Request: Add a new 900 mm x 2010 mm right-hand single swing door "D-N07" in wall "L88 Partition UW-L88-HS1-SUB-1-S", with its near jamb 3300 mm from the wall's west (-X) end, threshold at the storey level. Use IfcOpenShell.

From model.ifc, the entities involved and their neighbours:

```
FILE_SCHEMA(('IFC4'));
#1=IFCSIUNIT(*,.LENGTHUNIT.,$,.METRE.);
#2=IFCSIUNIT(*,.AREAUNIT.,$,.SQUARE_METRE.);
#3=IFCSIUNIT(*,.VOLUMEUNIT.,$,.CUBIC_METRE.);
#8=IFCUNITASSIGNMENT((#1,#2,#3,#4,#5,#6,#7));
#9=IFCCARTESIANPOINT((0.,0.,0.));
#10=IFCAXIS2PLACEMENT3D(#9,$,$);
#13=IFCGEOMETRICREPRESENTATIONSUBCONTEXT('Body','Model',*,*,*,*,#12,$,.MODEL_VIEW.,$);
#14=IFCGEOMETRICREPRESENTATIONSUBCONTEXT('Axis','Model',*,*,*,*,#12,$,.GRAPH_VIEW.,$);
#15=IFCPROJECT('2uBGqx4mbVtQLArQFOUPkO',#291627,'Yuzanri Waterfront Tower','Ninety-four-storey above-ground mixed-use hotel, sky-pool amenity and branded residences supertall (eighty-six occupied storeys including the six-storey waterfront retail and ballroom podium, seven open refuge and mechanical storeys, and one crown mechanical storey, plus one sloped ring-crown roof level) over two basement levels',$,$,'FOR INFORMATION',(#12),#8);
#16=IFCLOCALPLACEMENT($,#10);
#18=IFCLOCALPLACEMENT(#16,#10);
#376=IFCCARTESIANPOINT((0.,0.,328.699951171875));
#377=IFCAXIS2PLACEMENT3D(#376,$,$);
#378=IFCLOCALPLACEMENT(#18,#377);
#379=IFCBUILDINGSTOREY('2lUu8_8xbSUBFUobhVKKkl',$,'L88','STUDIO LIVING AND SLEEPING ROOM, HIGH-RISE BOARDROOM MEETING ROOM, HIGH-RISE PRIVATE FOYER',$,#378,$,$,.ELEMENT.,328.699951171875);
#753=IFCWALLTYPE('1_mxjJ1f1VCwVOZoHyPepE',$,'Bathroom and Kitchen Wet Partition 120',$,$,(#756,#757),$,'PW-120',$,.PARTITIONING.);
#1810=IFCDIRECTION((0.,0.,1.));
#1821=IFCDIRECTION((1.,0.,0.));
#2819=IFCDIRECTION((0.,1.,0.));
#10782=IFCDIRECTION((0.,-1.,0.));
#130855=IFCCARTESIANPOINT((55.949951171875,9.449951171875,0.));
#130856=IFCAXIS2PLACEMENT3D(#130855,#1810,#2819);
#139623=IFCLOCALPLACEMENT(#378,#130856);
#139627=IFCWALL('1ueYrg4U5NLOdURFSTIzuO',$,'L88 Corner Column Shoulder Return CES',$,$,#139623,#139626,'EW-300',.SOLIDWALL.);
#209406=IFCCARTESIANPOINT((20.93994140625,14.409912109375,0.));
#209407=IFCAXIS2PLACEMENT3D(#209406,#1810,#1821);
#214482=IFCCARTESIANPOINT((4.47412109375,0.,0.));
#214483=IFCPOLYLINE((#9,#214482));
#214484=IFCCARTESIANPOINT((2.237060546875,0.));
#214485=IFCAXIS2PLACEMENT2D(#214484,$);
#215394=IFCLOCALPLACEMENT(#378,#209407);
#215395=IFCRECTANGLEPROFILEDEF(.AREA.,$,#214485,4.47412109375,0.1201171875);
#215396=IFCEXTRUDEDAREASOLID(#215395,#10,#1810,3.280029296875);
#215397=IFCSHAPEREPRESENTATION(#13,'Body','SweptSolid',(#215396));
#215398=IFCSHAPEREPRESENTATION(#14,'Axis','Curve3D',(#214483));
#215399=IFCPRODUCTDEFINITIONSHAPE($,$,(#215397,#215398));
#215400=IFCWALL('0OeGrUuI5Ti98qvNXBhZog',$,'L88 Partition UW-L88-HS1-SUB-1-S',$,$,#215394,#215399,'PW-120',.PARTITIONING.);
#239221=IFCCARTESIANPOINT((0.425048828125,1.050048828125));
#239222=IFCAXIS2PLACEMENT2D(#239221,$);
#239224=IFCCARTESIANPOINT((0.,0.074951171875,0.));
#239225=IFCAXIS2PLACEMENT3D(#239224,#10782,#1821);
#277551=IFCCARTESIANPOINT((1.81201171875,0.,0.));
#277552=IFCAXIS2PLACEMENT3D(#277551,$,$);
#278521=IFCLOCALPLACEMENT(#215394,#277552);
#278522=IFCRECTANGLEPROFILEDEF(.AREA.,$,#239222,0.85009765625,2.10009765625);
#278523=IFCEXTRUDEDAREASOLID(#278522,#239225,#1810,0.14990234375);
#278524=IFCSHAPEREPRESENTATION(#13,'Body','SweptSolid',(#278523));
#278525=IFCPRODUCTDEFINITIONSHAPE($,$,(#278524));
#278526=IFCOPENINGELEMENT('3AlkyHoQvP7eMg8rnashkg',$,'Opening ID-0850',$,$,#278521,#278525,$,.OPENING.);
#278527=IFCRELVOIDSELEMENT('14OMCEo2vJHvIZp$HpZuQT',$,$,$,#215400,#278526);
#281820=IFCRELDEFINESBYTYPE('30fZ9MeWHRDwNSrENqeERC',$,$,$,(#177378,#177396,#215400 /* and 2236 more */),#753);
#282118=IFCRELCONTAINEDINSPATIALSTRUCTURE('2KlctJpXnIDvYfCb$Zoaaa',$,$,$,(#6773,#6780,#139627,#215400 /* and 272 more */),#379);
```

```python
import numpy as np
import ifcopenshell
import ifcopenshell.api.feature
import ifcopenshell.api.geometry
import ifcopenshell.api.root
import ifcopenshell.api.spatial
import ifcopenshell.geom
import ifcopenshell.util.element
import ifcopenshell.util.placement
import ifcopenshell.util.representation
import ifcopenshell.util.shape
import ifcopenshell.util.unit

model = ifcopenshell.open("model.ifc")
unit_scale = ifcopenshell.util.unit.calculate_unit_scale(model)
settings = ifcopenshell.geom.settings()


def volume(element):
    """Net volume in cubic metres, openings subtracted."""
    shape = ifcopenshell.geom.create_shape(settings, element)
    return ifcopenshell.util.shape.get_volume(shape.geometry)


wall = model.by_guid("0OeGrUuI5Ti98qvNXBhZog")
storey = ifcopenshell.util.element.get_container(wall, ifc_class="IfcBuildingStorey")
context = ifcopenshell.util.representation.get_context(model, "Model", "Body", "MODEL_VIEW")
before = volume(wall)

width, height, from_end, sill = 0.9, 2.01, 3.3, 0.0  # metres

# The wall runs along its own X axis, and the end named is its -X end.
wall_shape = ifcopenshell.geom.create_shape(settings, wall)
x, y, z = ifcopenshell.util.shape.get_vertices(wall_shape.geometry).T
start = x.min() + from_end
face, thickness = float(y.min()), float(y.max() - y.min())
wall_matrix = ifcopenshell.util.placement.get_local_placement(wall.ObjectPlacement)
level = ifcopenshell.util.placement.get_local_placement(storey.ObjectPlacement)[2, 3]


def in_wall(x, y):
    """Placement at x, y metres in the wall's axes, at sill height."""
    matrix = wall_matrix.copy()
    matrix[:, 3] = wall_matrix @ np.array([x / unit_scale, y / unit_scale, 0.0, 1.0])
    matrix[2, 3] = level + sill / unit_scale
    return matrix


# Opening: a box that overshoots both wall faces by 50 mm.
opening = ifcopenshell.api.root.create_entity(model, ifc_class="IfcOpeningElement", predefined_type="OPENING")
box = ifcopenshell.api.geometry.add_wall_representation(
    model, context=context, length=width, height=height, thickness=thickness + 0.1
)
ifcopenshell.api.geometry.assign_representation(model, product=opening, representation=box)
ifcopenshell.api.geometry.edit_object_placement(model, product=opening, matrix=in_wall(start, face - 0.05), is_si=False)
ifcopenshell.api.feature.add_feature(model, feature=opening, element=wall)

door = ifcopenshell.api.root.create_entity(model, ifc_class="IfcDoor", name="D-N07", predefined_type="DOOR")
door.OverallWidth, door.OverallHeight = width / unit_scale, height / unit_scale
door.OperationType = "SINGLE_SWING_RIGHT"
body = ifcopenshell.api.geometry.add_door_representation(
    model,
    context=context,
    overall_width=door.OverallWidth,
    overall_height=door.OverallHeight,
    operation_type="SINGLE_SWING_RIGHT",
    lining_properties={"LiningDepth": thickness / unit_scale, "ThresholdDepth": thickness / unit_scale},
)
ifcopenshell.api.geometry.assign_representation(model, product=door, representation=body)
ifcopenshell.api.spatial.assign_container(model, products=[door], relating_structure=storey)
ifcopenshell.api.feature.add_filling(model, opening=opening, element=door)

# The lining spans the wall, so the door starts at the wall face.
ifcopenshell.api.geometry.edit_object_placement(model, product=door, matrix=in_wall(start, face), is_si=False)

after = volume(wall)

print(f"wall volume {before:.3f} -> {after:.3f} m3")

model.write("model-out.ifc")
```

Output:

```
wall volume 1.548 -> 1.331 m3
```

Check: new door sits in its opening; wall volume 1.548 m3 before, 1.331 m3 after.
